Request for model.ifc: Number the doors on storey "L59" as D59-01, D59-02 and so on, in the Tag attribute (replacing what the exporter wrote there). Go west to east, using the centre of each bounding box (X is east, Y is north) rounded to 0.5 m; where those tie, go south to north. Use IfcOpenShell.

First a look at what the model holds.

```python
import ifcopenshell
import ifcopenshell.util.element
import ifcopenshell.util.placement

model = ifcopenshell.open("model.ifc")
print(model.schema)
storey = next(s for s in model.by_type("IfcBuildingStorey") if s.Name == "L59")
doors = [e for e in ifcopenshell.util.element.get_decomposition(storey) if e.is_a("IfcDoor")]
for e in sorted(doors, key=lambda e: e.id()):
    origin = ifcopenshell.util.placement.get_local_placement(e.ObjectPlacement)[:3, 3]
    print(e.id(), e.Tag, e.Name, origin.round(2) + 0.0, sep=" | ")
```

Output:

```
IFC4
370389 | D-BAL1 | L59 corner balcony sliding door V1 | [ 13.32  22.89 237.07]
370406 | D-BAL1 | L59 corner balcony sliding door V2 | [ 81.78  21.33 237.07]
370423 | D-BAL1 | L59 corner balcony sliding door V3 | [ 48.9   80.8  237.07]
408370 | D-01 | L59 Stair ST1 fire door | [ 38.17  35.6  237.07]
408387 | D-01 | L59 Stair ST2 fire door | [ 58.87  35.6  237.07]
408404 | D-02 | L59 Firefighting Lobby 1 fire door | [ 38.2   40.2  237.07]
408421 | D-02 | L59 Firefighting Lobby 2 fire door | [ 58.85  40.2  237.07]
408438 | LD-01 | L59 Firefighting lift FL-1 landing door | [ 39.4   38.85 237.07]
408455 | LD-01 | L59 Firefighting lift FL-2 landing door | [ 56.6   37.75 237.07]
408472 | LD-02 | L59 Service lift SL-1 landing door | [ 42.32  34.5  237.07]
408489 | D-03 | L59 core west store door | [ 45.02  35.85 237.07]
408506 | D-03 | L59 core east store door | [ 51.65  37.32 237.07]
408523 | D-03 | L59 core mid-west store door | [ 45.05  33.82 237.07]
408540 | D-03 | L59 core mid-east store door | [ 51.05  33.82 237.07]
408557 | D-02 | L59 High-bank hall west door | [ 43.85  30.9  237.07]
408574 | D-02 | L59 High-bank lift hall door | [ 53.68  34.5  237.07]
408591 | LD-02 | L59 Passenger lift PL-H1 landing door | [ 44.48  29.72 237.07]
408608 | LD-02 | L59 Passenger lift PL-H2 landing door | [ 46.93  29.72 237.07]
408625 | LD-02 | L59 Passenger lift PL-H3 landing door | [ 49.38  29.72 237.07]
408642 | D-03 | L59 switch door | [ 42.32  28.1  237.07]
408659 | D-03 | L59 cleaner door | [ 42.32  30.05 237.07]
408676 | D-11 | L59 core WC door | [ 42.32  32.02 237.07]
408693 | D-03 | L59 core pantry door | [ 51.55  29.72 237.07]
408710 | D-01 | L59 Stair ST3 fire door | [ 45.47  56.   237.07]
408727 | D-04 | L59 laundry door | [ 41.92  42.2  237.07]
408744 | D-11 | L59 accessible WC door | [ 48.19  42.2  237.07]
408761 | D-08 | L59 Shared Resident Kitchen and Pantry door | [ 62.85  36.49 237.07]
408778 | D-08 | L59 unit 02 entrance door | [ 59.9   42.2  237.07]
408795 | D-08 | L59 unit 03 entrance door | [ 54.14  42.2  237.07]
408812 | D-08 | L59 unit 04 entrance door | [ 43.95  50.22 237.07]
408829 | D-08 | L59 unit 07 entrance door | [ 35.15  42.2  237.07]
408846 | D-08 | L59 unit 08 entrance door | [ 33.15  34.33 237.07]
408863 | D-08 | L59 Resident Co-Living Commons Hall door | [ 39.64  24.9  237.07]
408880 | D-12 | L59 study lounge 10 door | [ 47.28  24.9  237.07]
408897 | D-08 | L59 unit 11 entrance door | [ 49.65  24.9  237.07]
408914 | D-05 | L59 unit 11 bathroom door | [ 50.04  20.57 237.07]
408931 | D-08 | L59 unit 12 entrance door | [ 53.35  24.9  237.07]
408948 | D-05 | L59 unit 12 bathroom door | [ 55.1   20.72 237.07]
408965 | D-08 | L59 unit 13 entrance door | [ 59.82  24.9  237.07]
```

```python
import ifcopenshell
import ifcopenshell.geom
import ifcopenshell.util.element
import ifcopenshell.util.shape

model = ifcopenshell.open("model.ifc")
settings = ifcopenshell.geom.settings()
settings.set("use-world-coords", True)


def centre(element):
    shape = ifcopenshell.geom.create_shape(settings, element)
    return ifcopenshell.util.shape.get_bbox_centroid(shape.geometry)


storey = next(s for s in model.by_type("IfcBuildingStorey") if s.Name == "L59")
doors = [e for e in ifcopenshell.util.element.get_decomposition(storey) if e.is_a("IfcDoor")]

# Insertion points can sit at a corner or the storey origin, so sort by the geometry (in metres).
centres = {e: centre(e) for e in doors}
doors.sort(key=lambda e: (round(centres[e][0] / 0.5), centres[e][1]))

for i, e in enumerate(doors, start=1):
    number = f"D59-{i:02d}"
    e.Tag = number
    print(e.id(), number)

model.write("model-out.ifc")
```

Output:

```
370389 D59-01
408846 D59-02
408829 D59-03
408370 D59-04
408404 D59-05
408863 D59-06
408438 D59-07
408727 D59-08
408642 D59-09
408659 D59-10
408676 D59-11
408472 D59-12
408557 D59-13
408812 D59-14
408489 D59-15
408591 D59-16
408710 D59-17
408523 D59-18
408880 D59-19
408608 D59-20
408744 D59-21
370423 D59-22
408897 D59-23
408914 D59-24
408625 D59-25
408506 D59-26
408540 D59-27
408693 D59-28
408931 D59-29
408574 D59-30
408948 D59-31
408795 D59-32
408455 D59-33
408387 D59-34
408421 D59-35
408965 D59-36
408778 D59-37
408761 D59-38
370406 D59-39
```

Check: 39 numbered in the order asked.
